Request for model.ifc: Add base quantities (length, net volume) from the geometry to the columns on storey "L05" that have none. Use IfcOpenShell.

First a look at what the model holds.

```python
import ifcopenshell
import ifcopenshell.util.element
import ifcopenshell.util.unit

model = ifcopenshell.open("model.ifc")
print(model.schema)
for unit_type in ("LENGTHUNIT", "AREAUNIT", "VOLUMEUNIT"):
    print(unit_type, ifcopenshell.util.unit.calculate_unit_scale(model, unit_type))
storey = next(s for s in model.by_type("IfcBuildingStorey") if s.Name == "L05")
columns = [e for e in ifcopenshell.util.element.get_decomposition(storey) if e.is_a("IfcColumn")]
for e in sorted(columns, key=lambda e: e.id()):
    print(e.id(), e.is_a(), e.Name, list(ifcopenshell.util.element.get_psets(e, qtos_only=True)), sep=" | ")
```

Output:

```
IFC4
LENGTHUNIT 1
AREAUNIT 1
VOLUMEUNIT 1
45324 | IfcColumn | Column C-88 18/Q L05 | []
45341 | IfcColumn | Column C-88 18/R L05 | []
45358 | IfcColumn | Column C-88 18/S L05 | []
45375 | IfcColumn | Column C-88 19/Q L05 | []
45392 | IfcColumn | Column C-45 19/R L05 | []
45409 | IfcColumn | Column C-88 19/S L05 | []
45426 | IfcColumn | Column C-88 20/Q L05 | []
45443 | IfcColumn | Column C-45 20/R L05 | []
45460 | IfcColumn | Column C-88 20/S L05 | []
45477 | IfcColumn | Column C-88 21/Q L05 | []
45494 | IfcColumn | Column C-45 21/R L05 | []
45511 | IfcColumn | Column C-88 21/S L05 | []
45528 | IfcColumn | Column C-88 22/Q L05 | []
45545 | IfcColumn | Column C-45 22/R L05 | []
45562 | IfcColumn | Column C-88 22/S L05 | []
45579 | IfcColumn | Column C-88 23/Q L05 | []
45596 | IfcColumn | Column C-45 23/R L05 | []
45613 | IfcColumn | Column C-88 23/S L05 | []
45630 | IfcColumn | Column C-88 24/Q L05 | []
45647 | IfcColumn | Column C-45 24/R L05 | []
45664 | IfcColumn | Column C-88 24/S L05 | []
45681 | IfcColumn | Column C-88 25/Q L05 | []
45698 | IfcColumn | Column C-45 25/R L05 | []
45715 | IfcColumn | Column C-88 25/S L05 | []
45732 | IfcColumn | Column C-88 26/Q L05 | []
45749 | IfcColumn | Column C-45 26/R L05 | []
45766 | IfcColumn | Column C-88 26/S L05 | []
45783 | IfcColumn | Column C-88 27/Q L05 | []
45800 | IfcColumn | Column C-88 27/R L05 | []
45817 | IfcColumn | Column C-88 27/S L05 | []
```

```python
import ifcopenshell
import ifcopenshell.api.pset
import ifcopenshell.geom
import ifcopenshell.util.element
import ifcopenshell.util.shape
import ifcopenshell.util.unit

model = ifcopenshell.open("model.ifc")
unit_scale = ifcopenshell.util.unit.calculate_unit_scale(model)
volume_scale = ifcopenshell.util.unit.calculate_unit_scale(model, "VOLUMEUNIT")
settings = ifcopenshell.geom.settings()

storey = next(s for s in model.by_type("IfcBuildingStorey") if s.Name == "L05")
columns = [e for e in ifcopenshell.util.element.get_decomposition(storey) if e.is_a("IfcColumn")]

for e in sorted(columns, key=lambda e: e.id()):
    if ifcopenshell.util.element.get_psets(e, qtos_only=True, should_inherit=False):
        continue
    # Geometry comes back in metres, in the element's own axes.
    shape = ifcopenshell.geom.create_shape(settings, e)
    values = {
        "Length": ifcopenshell.util.shape.get_z(shape.geometry) / unit_scale,
        "NetVolume": ifcopenshell.util.shape.get_volume(shape.geometry) / volume_scale,
    }
    qto = ifcopenshell.api.pset.add_qto(model, product=e, name="Qto_ColumnBaseQuantities")
    ifcopenshell.api.pset.edit_qto(model, qto=qto, properties=values)
    print(e.id(), {k: round(v, 3) for k, v in values.items()})

model.write("model_updated.ifc")
```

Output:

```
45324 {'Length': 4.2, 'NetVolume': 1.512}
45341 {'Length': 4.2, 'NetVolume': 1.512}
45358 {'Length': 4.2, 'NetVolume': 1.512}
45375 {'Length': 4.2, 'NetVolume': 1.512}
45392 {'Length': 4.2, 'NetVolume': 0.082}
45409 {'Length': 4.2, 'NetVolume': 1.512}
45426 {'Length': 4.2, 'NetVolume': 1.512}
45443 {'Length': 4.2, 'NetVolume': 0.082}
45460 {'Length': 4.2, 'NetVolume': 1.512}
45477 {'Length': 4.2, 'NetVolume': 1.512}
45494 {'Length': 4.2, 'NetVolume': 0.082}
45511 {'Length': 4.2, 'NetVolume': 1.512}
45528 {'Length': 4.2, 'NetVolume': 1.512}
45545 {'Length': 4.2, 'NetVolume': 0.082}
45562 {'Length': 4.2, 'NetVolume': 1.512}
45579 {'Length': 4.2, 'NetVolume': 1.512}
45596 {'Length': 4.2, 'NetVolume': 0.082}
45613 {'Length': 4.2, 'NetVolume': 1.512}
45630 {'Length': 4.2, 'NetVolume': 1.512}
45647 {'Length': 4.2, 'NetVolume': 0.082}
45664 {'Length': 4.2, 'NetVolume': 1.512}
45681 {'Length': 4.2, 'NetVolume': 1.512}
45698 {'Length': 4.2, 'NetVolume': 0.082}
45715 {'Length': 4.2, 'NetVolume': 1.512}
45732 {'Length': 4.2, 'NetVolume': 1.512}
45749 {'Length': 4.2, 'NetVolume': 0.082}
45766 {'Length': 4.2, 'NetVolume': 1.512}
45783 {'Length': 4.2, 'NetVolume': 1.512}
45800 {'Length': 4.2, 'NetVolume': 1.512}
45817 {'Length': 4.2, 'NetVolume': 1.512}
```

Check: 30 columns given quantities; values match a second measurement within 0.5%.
